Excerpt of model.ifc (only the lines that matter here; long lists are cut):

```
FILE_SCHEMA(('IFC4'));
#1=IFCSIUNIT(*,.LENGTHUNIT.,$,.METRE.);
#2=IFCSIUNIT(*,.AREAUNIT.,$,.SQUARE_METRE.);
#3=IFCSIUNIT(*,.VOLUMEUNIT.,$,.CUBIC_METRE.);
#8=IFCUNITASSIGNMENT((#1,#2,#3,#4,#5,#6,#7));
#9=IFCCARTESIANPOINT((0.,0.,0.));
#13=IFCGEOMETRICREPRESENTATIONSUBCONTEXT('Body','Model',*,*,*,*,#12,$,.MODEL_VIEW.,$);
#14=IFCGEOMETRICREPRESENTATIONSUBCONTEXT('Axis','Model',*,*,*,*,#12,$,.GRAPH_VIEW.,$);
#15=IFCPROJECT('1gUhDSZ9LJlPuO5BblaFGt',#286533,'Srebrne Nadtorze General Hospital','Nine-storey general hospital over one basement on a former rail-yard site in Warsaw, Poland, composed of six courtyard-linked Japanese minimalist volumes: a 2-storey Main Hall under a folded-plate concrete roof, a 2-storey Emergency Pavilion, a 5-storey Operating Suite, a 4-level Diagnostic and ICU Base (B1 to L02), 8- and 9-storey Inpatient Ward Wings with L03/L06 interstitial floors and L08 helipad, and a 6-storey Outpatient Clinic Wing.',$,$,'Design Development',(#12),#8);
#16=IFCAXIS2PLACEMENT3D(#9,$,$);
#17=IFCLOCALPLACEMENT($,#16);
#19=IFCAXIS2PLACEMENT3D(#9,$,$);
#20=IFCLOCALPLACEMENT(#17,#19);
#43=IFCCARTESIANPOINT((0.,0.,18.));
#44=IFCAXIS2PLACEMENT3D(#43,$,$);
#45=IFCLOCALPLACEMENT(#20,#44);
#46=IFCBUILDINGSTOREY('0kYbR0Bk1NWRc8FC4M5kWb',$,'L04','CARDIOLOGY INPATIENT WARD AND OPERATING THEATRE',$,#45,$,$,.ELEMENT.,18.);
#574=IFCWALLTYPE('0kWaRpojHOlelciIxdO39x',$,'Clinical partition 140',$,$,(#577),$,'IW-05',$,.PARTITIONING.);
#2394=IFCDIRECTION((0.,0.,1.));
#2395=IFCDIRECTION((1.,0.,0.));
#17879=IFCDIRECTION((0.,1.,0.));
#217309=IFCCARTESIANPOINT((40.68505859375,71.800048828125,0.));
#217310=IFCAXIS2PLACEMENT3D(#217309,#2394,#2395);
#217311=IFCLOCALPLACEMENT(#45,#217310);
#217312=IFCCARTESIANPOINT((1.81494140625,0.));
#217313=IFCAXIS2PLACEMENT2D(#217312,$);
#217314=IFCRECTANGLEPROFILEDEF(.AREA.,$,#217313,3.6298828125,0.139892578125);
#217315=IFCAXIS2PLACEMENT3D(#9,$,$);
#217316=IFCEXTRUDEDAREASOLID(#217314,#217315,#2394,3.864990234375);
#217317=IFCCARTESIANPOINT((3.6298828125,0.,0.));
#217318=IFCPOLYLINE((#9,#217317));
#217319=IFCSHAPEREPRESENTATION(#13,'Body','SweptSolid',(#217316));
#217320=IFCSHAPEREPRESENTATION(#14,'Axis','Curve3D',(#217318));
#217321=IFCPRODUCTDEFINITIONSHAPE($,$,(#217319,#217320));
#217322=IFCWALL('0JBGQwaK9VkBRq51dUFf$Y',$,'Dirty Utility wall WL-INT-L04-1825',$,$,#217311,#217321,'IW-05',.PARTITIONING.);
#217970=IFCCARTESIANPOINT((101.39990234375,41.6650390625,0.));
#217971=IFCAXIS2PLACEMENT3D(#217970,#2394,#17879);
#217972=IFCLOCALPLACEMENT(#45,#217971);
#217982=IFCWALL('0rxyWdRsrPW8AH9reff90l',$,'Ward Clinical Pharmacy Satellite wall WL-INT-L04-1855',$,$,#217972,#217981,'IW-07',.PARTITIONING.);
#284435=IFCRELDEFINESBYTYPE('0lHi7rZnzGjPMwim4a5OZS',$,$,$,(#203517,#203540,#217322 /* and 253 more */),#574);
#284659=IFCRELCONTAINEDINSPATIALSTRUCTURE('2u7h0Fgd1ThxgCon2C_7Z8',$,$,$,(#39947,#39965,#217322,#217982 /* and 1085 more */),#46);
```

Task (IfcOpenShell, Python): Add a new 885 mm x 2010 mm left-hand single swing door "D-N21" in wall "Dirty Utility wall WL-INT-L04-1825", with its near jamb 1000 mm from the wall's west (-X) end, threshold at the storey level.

```python
import numpy as np
import ifcopenshell
import ifcopenshell.api.feature
import ifcopenshell.api.geometry
import ifcopenshell.api.root
import ifcopenshell.api.spatial
import ifcopenshell.geom
import ifcopenshell.util.element
import ifcopenshell.util.placement
import ifcopenshell.util.representation
import ifcopenshell.util.shape
import ifcopenshell.util.unit

model = ifcopenshell.open("model.ifc")
unit_scale = ifcopenshell.util.unit.calculate_unit_scale(model)
settings = ifcopenshell.geom.settings()


def volume(element):
    """Net volume in cubic metres, openings subtracted."""
    shape = ifcopenshell.geom.create_shape(settings, element)
    return ifcopenshell.util.shape.get_volume(shape.geometry)


wall = model.by_guid("0JBGQwaK9VkBRq51dUFf$Y")
storey = ifcopenshell.util.element.get_container(wall, ifc_class="IfcBuildingStorey")
context = ifcopenshell.util.representation.get_context(model, "Model", "Body", "MODEL_VIEW")
before = volume(wall)

width, height, from_end, sill = 0.885, 2.01, 1, 0.0  # metres

# The wall runs along its own X axis, and the end named is its -X end.
wall_shape = ifcopenshell.geom.create_shape(settings, wall)
x, y, z = ifcopenshell.util.shape.get_vertices(wall_shape.geometry).T
start = x.min() + from_end
face, thickness = float(y.min()), float(y.max() - y.min())
wall_matrix = ifcopenshell.util.placement.get_local_placement(wall.ObjectPlacement)
level = ifcopenshell.util.placement.get_local_placement(storey.ObjectPlacement)[2, 3]


def in_wall(x, y):
    """Placement at x, y metres in the wall's axes, at sill height."""
    matrix = wall_matrix.copy()
    matrix[:, 3] = wall_matrix @ np.array([x / unit_scale, y / unit_scale, 0.0, 1.0])
    matrix[2, 3] = level + sill / unit_scale
    return matrix


# Opening: a box that overshoots both wall faces by 50 mm.
opening = ifcopenshell.api.root.create_entity(model, ifc_class="IfcOpeningElement", predefined_type="OPENING")
box = ifcopenshell.api.geometry.add_wall_representation(
    model, context=context, length=width, height=height, thickness=thickness + 0.1
)
ifcopenshell.api.geometry.assign_representation(model, product=opening, representation=box)
ifcopenshell.api.geometry.edit_object_placement(model, product=opening, matrix=in_wall(start, face - 0.05), is_si=False)
ifcopenshell.api.feature.add_feature(model, feature=opening, element=wall)

door = ifcopenshell.api.root.create_entity(model, ifc_class="IfcDoor", name="D-N21", predefined_type="DOOR")
door.OverallWidth, door.OverallHeight = width / unit_scale, height / unit_scale
door.OperationType = "SINGLE_SWING_LEFT"
body = ifcopenshell.api.geometry.add_door_representation(
    model,
    context=context,
    overall_width=door.OverallWidth,
    overall_height=door.OverallHeight,
    operation_type="SINGLE_SWING_LEFT",
    lining_properties={"LiningDepth": thickness / unit_scale, "ThresholdDepth": thickness / unit_scale},
)
ifcopenshell.api.geometry.assign_representation(model, product=door, representation=body)
ifcopenshell.api.spatial.assign_container(model, products=[door], relating_structure=storey)
ifcopenshell.api.feature.add_filling(model, opening=opening, element=door)

# The lining spans the wall, so the door starts at the wall face.
ifcopenshell.api.geometry.edit_object_placement(model, product=door, matrix=in_wall(start, face), is_si=False)

after = volume(wall)

print(f"wall volume {before:.3f} -> {after:.3f} m3")

model.write("model_edited.ifc")
```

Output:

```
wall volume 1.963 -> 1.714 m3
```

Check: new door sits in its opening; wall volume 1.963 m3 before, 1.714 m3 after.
